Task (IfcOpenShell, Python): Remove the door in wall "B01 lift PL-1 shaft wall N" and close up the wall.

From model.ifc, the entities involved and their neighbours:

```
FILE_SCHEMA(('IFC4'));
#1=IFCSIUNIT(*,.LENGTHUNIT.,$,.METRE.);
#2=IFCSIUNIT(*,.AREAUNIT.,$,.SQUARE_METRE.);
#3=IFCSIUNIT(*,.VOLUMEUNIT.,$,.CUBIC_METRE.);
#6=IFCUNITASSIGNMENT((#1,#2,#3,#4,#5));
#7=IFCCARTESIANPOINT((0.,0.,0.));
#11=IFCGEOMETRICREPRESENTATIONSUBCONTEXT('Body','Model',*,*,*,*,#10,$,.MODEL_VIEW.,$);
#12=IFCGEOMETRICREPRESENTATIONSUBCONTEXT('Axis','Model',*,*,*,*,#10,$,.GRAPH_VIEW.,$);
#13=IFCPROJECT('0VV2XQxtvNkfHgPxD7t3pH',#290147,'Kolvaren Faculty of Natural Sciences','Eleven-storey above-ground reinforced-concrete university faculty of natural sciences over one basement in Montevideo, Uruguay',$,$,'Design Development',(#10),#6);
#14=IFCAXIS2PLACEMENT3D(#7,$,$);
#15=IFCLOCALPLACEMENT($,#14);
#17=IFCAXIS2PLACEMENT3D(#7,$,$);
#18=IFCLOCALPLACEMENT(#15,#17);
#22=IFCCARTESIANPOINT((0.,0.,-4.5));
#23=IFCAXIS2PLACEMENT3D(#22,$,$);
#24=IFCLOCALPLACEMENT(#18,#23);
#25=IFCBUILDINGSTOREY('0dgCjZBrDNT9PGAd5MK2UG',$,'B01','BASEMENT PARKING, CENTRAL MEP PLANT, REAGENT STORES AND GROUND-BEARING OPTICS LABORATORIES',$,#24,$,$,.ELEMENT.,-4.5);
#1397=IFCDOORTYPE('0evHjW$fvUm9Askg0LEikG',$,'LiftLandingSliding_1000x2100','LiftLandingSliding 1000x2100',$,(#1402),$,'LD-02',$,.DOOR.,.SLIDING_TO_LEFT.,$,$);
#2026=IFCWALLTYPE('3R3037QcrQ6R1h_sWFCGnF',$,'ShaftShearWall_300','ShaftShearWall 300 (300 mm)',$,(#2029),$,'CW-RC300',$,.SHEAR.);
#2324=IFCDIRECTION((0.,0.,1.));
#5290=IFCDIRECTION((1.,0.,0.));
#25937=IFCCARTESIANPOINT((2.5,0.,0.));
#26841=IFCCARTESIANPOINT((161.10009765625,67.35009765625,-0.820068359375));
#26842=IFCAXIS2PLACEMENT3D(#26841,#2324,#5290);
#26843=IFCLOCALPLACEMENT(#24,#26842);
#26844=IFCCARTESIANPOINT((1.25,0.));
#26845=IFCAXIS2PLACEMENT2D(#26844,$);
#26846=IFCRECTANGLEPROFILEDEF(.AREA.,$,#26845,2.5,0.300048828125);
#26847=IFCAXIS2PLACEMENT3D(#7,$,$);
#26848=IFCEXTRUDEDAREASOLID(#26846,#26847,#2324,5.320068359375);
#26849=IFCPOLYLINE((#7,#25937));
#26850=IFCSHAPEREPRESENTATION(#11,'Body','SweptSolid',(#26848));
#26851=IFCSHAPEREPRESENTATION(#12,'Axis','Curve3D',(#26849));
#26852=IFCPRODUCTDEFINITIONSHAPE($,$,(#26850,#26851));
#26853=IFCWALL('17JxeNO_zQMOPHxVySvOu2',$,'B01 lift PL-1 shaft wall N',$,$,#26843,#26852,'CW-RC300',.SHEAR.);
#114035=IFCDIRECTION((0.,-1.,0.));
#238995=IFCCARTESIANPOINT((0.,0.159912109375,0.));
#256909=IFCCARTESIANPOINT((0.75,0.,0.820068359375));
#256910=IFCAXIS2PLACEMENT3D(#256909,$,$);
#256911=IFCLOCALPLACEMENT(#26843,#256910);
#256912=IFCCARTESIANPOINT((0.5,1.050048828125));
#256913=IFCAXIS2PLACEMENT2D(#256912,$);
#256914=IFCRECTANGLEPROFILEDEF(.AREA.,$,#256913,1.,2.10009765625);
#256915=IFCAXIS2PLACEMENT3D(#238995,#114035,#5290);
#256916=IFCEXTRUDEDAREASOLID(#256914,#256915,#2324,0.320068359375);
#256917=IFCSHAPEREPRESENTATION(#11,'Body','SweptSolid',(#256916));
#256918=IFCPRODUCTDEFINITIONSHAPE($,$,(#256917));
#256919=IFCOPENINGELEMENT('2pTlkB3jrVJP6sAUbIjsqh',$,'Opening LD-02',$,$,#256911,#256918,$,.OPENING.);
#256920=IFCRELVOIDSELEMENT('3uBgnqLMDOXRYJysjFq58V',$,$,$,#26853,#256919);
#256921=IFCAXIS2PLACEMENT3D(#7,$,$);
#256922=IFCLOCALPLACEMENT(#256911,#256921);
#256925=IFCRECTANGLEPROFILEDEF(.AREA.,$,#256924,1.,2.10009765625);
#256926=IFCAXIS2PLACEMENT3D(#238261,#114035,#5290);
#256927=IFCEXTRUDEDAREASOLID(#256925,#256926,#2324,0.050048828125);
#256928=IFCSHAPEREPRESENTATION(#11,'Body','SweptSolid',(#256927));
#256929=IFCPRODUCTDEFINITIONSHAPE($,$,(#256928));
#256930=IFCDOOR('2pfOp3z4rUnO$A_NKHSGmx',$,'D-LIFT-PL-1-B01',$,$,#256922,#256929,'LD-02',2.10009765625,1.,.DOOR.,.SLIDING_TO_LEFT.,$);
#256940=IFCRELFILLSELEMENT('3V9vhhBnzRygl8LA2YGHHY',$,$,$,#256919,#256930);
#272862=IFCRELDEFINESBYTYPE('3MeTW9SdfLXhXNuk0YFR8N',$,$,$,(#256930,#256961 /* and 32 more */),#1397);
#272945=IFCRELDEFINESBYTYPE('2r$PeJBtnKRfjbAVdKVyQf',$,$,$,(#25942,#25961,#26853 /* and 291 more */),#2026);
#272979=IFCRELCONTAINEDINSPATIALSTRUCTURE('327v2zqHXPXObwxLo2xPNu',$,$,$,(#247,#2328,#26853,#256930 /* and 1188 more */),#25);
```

```python
import ifcopenshell
import ifcopenshell.api.feature
import ifcopenshell.api.root
import ifcopenshell.geom
import ifcopenshell.util.shape

model = ifcopenshell.open("model.ifc")
settings = ifcopenshell.geom.settings()


def volume(element):
    """Net volume in cubic metres, openings subtracted."""
    shape = ifcopenshell.geom.create_shape(settings, element)
    return ifcopenshell.util.shape.get_volume(shape.geometry)


door = model.by_guid("2pfOp3z4rUnO$A_NKHSGmx")
opening = door.FillsVoids[0].RelatingOpeningElement
wall = opening.VoidsElements[0].RelatingBuildingElement
before = volume(wall)

ifcopenshell.api.root.remove_product(model, product=door)
ifcopenshell.api.feature.remove_feature(model, feature=opening)

after = volume(wall)

print(f"wall volume {before:.3f} -> {after:.3f} m3")

model.write("model_edited.ifc")
```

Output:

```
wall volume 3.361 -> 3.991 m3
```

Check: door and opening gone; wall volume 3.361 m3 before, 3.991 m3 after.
